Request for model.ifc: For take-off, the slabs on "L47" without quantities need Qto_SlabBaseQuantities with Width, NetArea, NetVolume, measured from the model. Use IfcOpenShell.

First a look at what the model holds.

```python
import ifcopenshell
import ifcopenshell.util.element
import ifcopenshell.util.unit

model = ifcopenshell.open("model.ifc")
print(model.schema)
for unit_type in ("LENGTHUNIT", "AREAUNIT", "VOLUMEUNIT"):
    print(unit_type, ifcopenshell.util.unit.calculate_unit_scale(model, unit_type))
storey = next(s for s in model.by_type("IfcBuildingStorey") if s.Name == "L47")
slabs = [e for e in ifcopenshell.util.element.get_decomposition(storey) if e.is_a("IfcSlab")]
for e in sorted(slabs, key=lambda e: e.id()):
    print(e.id(), e.is_a(), e.Name, list(ifcopenshell.util.element.get_psets(e, qtos_only=True)), sep=" | ")
```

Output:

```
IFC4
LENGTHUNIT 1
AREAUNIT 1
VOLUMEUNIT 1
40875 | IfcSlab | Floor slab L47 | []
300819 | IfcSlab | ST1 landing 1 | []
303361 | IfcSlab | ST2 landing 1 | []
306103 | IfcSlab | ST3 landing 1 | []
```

```python
import ifcopenshell
import ifcopenshell.api.pset
import ifcopenshell.geom
import ifcopenshell.util.element
import ifcopenshell.util.shape
import ifcopenshell.util.unit

model = ifcopenshell.open("model.ifc")
unit_scale = ifcopenshell.util.unit.calculate_unit_scale(model)
area_scale = ifcopenshell.util.unit.calculate_unit_scale(model, "AREAUNIT")
volume_scale = ifcopenshell.util.unit.calculate_unit_scale(model, "VOLUMEUNIT")
settings = ifcopenshell.geom.settings()

storey = next(s for s in model.by_type("IfcBuildingStorey") if s.Name == "L47")
slabs = [e for e in ifcopenshell.util.element.get_decomposition(storey) if e.is_a("IfcSlab")]

for e in sorted(slabs, key=lambda e: e.id()):
    if ifcopenshell.util.element.get_psets(e, qtos_only=True, should_inherit=False):
        continue
    # Geometry comes back in metres, in the element's own axes.
    shape = ifcopenshell.geom.create_shape(settings, e)
    values = {
        "Width": ifcopenshell.util.shape.get_z(shape.geometry) / unit_scale,
        "NetArea": ifcopenshell.util.shape.get_footprint_area(shape.geometry) / area_scale,
        "NetVolume": ifcopenshell.util.shape.get_volume(shape.geometry) / volume_scale,
    }
    qto = ifcopenshell.api.pset.add_qto(model, product=e, name="Qto_SlabBaseQuantities")
    ifcopenshell.api.pset.edit_qto(model, qto=qto, properties=values)
    print(e.id(), {k: round(v, 3) for k, v in values.items()})

model.write("model_v2.ifc")
```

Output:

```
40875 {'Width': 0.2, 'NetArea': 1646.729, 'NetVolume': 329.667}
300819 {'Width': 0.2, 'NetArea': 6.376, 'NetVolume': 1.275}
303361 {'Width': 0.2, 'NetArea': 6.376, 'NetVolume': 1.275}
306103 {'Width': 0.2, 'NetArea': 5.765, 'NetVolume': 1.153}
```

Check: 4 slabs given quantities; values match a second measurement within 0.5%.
